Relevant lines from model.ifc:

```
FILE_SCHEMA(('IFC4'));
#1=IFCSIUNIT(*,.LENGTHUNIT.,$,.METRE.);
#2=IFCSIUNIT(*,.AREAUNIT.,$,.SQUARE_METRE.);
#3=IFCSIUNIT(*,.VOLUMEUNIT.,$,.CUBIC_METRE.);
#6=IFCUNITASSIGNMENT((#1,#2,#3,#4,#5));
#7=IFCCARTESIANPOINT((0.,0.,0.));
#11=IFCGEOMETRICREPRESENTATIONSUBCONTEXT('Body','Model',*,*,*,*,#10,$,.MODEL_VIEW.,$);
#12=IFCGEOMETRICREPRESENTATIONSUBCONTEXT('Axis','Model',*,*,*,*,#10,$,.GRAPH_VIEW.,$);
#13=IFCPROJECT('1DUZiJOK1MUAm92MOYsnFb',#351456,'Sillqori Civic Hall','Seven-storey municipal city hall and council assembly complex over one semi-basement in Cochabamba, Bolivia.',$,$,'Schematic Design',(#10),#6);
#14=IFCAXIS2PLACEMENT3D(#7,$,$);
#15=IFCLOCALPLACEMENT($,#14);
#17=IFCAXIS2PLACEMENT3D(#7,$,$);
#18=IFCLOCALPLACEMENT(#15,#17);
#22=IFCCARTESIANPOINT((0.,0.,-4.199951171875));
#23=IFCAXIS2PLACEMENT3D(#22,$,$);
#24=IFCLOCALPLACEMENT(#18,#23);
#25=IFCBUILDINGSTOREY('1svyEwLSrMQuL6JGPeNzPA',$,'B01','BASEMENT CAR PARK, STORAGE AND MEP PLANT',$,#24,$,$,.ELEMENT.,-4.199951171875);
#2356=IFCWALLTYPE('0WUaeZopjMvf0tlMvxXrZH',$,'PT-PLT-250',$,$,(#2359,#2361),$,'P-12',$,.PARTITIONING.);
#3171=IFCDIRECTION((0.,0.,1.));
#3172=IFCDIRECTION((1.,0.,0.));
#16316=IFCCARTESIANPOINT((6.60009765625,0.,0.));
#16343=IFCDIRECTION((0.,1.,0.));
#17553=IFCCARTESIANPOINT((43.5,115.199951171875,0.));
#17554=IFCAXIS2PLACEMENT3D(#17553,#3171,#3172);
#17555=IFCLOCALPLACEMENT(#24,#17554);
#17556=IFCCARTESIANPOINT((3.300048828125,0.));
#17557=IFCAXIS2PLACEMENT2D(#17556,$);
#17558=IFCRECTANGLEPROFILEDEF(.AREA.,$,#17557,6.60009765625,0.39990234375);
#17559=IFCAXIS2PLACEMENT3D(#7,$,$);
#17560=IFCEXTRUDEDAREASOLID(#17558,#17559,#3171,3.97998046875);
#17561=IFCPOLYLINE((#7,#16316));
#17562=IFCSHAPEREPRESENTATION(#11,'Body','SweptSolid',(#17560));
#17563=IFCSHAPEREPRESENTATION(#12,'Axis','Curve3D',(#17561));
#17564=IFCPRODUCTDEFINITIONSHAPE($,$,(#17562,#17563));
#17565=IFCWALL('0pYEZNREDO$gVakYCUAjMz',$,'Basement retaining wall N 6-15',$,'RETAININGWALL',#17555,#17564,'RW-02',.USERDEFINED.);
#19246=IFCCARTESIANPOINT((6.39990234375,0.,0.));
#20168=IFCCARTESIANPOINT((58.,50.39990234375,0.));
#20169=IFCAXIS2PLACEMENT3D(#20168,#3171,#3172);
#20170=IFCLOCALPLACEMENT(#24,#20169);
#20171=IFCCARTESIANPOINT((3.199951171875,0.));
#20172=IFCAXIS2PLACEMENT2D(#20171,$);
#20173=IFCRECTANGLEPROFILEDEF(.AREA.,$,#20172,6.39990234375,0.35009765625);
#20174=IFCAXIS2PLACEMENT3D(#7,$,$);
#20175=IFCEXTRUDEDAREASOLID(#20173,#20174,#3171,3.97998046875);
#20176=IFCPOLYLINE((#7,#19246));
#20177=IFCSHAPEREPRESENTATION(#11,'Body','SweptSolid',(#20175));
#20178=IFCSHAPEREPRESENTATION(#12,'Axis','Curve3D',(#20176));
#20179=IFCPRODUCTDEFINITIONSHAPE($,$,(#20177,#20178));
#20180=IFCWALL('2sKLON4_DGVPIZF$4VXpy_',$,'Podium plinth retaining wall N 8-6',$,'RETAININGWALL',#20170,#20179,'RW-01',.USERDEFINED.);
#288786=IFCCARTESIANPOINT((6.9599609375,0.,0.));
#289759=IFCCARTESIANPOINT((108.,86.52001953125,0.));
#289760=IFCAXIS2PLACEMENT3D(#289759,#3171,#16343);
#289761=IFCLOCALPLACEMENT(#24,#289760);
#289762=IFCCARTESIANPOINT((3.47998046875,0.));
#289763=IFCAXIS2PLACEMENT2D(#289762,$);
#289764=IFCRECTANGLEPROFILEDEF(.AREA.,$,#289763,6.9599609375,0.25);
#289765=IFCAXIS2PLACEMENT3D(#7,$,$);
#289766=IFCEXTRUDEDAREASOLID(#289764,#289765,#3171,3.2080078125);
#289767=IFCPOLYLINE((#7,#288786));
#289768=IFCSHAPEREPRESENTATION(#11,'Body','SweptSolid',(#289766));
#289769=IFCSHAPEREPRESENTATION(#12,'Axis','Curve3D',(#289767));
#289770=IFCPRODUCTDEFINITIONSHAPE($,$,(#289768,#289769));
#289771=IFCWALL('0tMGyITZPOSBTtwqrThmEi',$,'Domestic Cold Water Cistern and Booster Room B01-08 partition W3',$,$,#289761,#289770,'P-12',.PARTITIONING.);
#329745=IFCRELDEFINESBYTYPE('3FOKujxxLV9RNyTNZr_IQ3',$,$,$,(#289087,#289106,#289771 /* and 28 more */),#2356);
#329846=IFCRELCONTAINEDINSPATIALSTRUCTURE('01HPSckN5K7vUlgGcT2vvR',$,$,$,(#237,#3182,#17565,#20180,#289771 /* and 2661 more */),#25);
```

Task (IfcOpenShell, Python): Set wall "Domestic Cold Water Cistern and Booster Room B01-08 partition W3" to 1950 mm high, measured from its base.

```python
import ifcopenshell
import ifcopenshell.geom
import ifcopenshell.util.representation
import ifcopenshell.util.shape

model = ifcopenshell.open("model.ifc")
settings = ifcopenshell.geom.settings()


def volume(element):
    """Net volume in cubic metres, openings subtracted."""
    shape = ifcopenshell.geom.create_shape(settings, element)
    return ifcopenshell.util.shape.get_volume(shape.geometry)


wall = model.by_id(289771)
before = volume(wall)

body = ifcopenshell.util.representation.get_representation(wall, "Model", "Body")
solid = body.Items[0]
old_height = solid.Depth
solid.Depth = 1.95
after = volume(wall)

print(f"height {old_height:g} -> {solid.Depth:g}, volume {before:.3f} -> {after:.3f} m3")

model.write("model_edited.ifc")
```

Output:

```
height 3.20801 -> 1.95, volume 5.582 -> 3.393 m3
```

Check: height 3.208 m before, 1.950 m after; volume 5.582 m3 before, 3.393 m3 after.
